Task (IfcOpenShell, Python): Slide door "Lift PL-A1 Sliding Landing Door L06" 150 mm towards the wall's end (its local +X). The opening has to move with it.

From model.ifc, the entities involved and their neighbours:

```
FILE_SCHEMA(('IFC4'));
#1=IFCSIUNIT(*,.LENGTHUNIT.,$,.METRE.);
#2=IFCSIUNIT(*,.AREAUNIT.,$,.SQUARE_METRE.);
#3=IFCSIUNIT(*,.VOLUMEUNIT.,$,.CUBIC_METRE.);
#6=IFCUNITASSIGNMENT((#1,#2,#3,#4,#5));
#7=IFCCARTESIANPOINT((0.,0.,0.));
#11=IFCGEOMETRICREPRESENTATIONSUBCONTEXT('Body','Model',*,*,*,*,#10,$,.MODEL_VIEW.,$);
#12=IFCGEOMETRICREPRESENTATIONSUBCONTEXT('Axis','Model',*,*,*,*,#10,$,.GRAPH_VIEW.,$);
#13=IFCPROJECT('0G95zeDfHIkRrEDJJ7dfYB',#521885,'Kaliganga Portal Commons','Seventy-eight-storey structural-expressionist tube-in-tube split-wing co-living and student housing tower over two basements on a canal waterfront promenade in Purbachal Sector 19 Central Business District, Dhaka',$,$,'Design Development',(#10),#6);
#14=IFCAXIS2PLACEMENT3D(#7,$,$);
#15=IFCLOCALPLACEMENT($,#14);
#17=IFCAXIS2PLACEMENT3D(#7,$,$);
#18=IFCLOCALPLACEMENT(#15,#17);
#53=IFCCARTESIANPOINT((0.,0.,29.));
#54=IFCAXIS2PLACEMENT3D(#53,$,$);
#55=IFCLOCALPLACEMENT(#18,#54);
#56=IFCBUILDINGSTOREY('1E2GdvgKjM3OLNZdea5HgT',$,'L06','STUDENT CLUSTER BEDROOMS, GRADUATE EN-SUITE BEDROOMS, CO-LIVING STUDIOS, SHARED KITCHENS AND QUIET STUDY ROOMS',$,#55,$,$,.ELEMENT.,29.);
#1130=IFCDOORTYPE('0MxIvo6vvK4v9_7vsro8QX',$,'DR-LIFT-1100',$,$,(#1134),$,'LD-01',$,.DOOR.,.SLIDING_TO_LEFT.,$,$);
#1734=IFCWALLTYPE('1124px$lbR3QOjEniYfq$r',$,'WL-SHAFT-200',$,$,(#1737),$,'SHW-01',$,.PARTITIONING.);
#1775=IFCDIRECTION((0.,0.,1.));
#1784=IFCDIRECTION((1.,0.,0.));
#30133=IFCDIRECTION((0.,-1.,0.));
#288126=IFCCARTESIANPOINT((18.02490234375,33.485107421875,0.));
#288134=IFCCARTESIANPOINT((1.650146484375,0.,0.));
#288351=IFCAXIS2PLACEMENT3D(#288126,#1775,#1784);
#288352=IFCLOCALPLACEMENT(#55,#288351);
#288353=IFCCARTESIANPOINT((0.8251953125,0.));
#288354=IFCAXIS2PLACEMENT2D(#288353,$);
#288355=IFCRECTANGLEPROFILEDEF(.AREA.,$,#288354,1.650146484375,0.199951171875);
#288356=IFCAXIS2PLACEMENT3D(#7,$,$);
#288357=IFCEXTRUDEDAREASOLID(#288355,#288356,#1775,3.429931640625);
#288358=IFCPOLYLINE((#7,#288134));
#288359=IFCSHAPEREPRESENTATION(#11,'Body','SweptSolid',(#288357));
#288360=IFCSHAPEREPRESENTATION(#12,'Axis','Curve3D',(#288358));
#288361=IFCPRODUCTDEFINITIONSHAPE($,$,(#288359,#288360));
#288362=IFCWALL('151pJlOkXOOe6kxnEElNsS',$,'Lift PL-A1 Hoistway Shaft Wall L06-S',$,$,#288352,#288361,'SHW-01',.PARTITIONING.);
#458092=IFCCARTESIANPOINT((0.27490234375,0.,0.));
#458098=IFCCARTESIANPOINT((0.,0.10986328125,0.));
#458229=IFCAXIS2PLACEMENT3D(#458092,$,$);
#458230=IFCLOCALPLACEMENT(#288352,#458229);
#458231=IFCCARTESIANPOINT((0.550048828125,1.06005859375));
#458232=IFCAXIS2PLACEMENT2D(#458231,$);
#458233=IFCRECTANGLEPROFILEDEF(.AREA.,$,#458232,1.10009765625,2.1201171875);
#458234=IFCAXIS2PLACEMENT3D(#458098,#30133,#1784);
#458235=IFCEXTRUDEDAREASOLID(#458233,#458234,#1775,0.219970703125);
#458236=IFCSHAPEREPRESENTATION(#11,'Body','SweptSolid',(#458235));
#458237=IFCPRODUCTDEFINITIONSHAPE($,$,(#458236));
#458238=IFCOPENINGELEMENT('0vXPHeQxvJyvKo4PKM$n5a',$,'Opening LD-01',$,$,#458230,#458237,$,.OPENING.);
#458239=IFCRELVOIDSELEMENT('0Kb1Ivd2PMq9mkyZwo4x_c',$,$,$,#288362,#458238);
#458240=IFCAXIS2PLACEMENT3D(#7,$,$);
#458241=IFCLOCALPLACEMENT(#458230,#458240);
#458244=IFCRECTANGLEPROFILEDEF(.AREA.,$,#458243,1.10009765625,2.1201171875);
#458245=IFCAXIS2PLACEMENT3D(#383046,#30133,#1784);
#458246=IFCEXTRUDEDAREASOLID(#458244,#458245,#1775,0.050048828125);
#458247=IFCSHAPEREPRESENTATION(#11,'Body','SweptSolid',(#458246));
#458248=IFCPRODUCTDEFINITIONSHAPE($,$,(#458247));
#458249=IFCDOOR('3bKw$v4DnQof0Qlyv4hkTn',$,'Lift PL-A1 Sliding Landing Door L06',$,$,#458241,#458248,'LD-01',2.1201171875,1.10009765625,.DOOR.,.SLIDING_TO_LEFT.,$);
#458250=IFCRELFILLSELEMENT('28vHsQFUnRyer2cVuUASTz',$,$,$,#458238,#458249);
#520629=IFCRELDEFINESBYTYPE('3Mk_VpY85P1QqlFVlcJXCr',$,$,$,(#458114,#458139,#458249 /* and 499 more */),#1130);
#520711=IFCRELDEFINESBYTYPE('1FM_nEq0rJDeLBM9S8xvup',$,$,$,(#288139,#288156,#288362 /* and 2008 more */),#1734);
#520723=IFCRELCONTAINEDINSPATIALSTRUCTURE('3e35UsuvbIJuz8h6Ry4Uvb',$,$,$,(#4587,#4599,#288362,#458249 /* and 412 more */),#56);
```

```python
import ifcopenshell
import ifcopenshell.api.geometry
import ifcopenshell.util.placement
import ifcopenshell.util.unit

model = ifcopenshell.open("model.ifc")
unit_scale = ifcopenshell.util.unit.calculate_unit_scale(model)

door = model.by_guid("3bKw$v4DnQof0Qlyv4hkTn")
opening = door.FillsVoids[0].RelatingOpeningElement
wall = opening.VoidsElements[0].RelatingBuildingElement

wall_matrix = ifcopenshell.util.placement.get_local_placement(wall.ObjectPlacement)
shift = wall_matrix[:3, 0] * 0.15 / unit_scale
before = ifcopenshell.util.placement.get_local_placement(door.ObjectPlacement)[:3, 3].copy()

# The door is placed relative to its opening, so it follows when the opening moves.
matrix = ifcopenshell.util.placement.get_local_placement(opening.ObjectPlacement)
matrix[:3, 3] += shift
ifcopenshell.api.geometry.edit_object_placement(
    model, product=opening, matrix=matrix, is_si=False, should_transform_children=True
)

after = ifcopenshell.util.placement.get_local_placement(door.ObjectPlacement)[:3, 3]
print("door moved by", (after - before).round(3) + 0.0)

model.write("model_rev.ifc")
```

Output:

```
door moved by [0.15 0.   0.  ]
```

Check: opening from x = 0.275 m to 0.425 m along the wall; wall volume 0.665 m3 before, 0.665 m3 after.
